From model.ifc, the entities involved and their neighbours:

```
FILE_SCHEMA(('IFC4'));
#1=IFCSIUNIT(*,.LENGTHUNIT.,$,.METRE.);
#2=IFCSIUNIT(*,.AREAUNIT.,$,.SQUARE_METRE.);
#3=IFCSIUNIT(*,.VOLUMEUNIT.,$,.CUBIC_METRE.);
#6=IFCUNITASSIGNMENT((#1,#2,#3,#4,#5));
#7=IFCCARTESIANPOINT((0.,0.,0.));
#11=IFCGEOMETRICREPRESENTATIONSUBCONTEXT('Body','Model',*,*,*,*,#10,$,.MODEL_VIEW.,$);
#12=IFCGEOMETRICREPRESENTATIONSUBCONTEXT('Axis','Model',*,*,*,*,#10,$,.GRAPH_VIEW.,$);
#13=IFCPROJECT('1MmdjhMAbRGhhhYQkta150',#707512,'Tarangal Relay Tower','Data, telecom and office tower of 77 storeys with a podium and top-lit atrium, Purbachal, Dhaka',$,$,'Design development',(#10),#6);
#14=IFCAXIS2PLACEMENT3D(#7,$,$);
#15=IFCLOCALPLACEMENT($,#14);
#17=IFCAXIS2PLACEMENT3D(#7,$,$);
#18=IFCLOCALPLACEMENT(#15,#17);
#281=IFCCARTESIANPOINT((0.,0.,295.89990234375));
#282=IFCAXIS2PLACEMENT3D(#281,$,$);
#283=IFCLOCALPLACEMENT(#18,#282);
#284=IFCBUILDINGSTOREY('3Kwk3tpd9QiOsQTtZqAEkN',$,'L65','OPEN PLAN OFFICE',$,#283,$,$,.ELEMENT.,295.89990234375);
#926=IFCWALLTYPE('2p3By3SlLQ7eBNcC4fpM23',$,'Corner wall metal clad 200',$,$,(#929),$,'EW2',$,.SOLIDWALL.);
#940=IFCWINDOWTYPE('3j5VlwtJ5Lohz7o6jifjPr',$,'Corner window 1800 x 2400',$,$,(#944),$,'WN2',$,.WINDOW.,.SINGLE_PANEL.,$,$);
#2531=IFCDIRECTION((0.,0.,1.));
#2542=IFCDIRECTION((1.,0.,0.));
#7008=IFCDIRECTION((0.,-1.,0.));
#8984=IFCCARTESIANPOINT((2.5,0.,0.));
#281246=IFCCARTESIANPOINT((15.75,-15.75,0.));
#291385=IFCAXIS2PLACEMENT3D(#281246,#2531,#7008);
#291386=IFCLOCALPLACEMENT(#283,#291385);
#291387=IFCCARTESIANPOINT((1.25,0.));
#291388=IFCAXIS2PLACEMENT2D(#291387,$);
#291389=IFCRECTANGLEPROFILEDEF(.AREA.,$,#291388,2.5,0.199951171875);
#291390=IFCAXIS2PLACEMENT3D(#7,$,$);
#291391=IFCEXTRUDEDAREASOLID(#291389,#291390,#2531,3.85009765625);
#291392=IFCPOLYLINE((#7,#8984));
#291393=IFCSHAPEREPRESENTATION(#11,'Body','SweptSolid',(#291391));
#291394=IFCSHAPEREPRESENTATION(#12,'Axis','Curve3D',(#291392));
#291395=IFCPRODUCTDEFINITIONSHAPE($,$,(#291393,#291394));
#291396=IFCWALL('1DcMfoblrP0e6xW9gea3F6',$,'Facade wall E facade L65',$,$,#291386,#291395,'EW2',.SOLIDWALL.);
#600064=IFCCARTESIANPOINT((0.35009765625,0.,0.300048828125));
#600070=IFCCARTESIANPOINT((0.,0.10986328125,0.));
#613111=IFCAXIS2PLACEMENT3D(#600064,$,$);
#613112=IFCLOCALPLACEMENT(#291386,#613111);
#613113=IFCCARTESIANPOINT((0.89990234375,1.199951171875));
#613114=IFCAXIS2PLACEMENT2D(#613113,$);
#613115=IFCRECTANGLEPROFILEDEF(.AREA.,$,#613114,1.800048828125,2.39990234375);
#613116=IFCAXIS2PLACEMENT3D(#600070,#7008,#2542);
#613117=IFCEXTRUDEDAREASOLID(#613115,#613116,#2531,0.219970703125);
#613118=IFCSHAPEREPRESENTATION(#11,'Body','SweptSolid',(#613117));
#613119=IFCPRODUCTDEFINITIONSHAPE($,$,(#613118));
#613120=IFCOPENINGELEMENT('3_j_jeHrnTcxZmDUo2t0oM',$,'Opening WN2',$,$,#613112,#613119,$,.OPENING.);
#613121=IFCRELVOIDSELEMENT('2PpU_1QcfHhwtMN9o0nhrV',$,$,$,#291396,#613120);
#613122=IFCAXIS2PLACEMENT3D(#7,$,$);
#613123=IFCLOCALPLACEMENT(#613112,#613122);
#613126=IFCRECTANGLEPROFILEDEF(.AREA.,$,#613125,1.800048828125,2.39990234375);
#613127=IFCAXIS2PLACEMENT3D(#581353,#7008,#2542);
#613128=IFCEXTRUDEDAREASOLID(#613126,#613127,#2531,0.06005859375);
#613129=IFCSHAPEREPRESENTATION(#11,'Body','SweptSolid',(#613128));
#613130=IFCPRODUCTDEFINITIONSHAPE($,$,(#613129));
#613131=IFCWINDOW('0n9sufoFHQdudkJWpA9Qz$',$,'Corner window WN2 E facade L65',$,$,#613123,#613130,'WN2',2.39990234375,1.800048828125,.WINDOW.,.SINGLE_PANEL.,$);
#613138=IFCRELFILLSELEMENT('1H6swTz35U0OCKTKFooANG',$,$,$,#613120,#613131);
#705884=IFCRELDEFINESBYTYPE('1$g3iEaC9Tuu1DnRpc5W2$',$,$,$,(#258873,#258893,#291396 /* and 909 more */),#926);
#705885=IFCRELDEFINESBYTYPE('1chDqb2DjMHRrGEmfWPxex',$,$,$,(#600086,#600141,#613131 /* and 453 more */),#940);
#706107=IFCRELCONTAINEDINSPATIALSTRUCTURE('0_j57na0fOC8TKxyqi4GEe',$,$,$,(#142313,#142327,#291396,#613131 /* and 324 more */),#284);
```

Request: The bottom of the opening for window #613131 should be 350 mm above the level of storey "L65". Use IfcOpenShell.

```python
import numpy as np
import ifcopenshell
import ifcopenshell.api.geometry
import ifcopenshell.geom
import ifcopenshell.util.element
import ifcopenshell.util.placement
import ifcopenshell.util.shape
import ifcopenshell.util.unit

model = ifcopenshell.open("model.ifc")
unit_scale = ifcopenshell.util.unit.calculate_unit_scale(model)

window = model.by_guid("0n9sufoFHQdudkJWpA9Qz$")
opening = window.FillsVoids[0].RelatingOpeningElement
storey = ifcopenshell.util.element.get_container(window, ifc_class="IfcBuildingStorey")
level = ifcopenshell.util.placement.get_local_placement(storey.ObjectPlacement)[2, 3]

# The opening's origin need not be at the sill, so measure its lowest point.
shape = ifcopenshell.geom.create_shape(ifcopenshell.geom.settings(), opening)
bottom = ifcopenshell.util.shape.get_shape_bottom_elevation(shape, shape.geometry) / unit_scale
dz = level + 0.35 - bottom

shift = np.array([0.0, 0.0, dz])
# The window is placed relative to its opening, so it follows when the opening moves.
matrix = ifcopenshell.util.placement.get_local_placement(opening.ObjectPlacement)
matrix[:3, 3] += shift
ifcopenshell.api.geometry.edit_object_placement(
    model, product=opening, matrix=matrix, is_si=False, should_transform_children=True
)

print(f"moved by {dz * unit_scale:+.3f} m")

model.write("model_v2.ifc")
```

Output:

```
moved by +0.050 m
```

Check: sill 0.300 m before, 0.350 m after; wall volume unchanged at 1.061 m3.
